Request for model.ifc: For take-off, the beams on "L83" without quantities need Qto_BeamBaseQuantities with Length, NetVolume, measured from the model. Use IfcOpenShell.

First a look at what the model holds.

```python
import ifcopenshell
import ifcopenshell.util.element
import ifcopenshell.util.unit

model = ifcopenshell.open("model.ifc")
print(model.schema)
for unit_type in ("LENGTHUNIT", "AREAUNIT", "VOLUMEUNIT"):
    print(unit_type, ifcopenshell.util.unit.calculate_unit_scale(model, unit_type))
storey = next(s for s in model.by_type("IfcBuildingStorey") if s.Name == "L83")
beams = [e for e in ifcopenshell.util.element.get_decomposition(storey) if e.is_a("IfcBeam")]
for e in sorted(beams, key=lambda e: e.id()):
    print(e.id(), e.is_a(), e.Name, list(ifcopenshell.util.element.get_psets(e, qtos_only=True)), sep=" | ")
```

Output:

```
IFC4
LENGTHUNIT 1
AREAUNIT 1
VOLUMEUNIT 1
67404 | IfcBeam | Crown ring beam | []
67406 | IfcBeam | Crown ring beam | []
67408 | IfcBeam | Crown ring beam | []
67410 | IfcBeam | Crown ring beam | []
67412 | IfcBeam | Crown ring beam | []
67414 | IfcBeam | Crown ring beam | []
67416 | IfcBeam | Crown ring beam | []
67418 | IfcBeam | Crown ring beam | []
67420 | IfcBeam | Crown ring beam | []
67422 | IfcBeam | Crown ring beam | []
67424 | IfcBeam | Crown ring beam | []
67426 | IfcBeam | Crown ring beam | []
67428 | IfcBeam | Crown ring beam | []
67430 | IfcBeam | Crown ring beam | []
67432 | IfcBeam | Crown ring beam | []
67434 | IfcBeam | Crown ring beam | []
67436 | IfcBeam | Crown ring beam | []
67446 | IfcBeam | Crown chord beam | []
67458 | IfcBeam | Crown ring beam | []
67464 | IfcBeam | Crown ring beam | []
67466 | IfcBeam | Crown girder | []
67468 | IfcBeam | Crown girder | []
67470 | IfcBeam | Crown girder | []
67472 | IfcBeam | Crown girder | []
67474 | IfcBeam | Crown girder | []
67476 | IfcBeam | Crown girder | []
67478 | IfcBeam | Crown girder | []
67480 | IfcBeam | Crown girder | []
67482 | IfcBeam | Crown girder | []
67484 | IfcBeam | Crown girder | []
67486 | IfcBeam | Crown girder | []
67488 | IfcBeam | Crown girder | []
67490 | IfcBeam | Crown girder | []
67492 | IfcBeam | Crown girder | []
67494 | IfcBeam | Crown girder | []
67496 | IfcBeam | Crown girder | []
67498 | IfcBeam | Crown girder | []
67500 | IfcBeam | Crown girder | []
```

```python
import ifcopenshell
import ifcopenshell.api.pset
import ifcopenshell.geom
import ifcopenshell.util.element
import ifcopenshell.util.shape
import ifcopenshell.util.unit

model = ifcopenshell.open("model.ifc")
unit_scale = ifcopenshell.util.unit.calculate_unit_scale(model)
volume_scale = ifcopenshell.util.unit.calculate_unit_scale(model, "VOLUMEUNIT")
settings = ifcopenshell.geom.settings()

storey = next(s for s in model.by_type("IfcBuildingStorey") if s.Name == "L83")
beams = [e for e in ifcopenshell.util.element.get_decomposition(storey) if e.is_a("IfcBeam")]

for e in sorted(beams, key=lambda e: e.id()):
    if ifcopenshell.util.element.get_psets(e, qtos_only=True, should_inherit=False):
        continue
    # Geometry comes back in metres, in the element's own axes.
    shape = ifcopenshell.geom.create_shape(settings, e)
    values = {
        "Length": ifcopenshell.util.shape.get_max_xyz(shape.geometry) / unit_scale,
        "NetVolume": ifcopenshell.util.shape.get_volume(shape.geometry) / volume_scale,
    }
    qto = ifcopenshell.api.pset.add_qto(model, product=e, name="Qto_BeamBaseQuantities")
    ifcopenshell.api.pset.edit_qto(model, qto=qto, properties=values)
    print(e.id(), {k: round(v, 3) for k, v in values.items()})

model.write("model_edited.ifc")
```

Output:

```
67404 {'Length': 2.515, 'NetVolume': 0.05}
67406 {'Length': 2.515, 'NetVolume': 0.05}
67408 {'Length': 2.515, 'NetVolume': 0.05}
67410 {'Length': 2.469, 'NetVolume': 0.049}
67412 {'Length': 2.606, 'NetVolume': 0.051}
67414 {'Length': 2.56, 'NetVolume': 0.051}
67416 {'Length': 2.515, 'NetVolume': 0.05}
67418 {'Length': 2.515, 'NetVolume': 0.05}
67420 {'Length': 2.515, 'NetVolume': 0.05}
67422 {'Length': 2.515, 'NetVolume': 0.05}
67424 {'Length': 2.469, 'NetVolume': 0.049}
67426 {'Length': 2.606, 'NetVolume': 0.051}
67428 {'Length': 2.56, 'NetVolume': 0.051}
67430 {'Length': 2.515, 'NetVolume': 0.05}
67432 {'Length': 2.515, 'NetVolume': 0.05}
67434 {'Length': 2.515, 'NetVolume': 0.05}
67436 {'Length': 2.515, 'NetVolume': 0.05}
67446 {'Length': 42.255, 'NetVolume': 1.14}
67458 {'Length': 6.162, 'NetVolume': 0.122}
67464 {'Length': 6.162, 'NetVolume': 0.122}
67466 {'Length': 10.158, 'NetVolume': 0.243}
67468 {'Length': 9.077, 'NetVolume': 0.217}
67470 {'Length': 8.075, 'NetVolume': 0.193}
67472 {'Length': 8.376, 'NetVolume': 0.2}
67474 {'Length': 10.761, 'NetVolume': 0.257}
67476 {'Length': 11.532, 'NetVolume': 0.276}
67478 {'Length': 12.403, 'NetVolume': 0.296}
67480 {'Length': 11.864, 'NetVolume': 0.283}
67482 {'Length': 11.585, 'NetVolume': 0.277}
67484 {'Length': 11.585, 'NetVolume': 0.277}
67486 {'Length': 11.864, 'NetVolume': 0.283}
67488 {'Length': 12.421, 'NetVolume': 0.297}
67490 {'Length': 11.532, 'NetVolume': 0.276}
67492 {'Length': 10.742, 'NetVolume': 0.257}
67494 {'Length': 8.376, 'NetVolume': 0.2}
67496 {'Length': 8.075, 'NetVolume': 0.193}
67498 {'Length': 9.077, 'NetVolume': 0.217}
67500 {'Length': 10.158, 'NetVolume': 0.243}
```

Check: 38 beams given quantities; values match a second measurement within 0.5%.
